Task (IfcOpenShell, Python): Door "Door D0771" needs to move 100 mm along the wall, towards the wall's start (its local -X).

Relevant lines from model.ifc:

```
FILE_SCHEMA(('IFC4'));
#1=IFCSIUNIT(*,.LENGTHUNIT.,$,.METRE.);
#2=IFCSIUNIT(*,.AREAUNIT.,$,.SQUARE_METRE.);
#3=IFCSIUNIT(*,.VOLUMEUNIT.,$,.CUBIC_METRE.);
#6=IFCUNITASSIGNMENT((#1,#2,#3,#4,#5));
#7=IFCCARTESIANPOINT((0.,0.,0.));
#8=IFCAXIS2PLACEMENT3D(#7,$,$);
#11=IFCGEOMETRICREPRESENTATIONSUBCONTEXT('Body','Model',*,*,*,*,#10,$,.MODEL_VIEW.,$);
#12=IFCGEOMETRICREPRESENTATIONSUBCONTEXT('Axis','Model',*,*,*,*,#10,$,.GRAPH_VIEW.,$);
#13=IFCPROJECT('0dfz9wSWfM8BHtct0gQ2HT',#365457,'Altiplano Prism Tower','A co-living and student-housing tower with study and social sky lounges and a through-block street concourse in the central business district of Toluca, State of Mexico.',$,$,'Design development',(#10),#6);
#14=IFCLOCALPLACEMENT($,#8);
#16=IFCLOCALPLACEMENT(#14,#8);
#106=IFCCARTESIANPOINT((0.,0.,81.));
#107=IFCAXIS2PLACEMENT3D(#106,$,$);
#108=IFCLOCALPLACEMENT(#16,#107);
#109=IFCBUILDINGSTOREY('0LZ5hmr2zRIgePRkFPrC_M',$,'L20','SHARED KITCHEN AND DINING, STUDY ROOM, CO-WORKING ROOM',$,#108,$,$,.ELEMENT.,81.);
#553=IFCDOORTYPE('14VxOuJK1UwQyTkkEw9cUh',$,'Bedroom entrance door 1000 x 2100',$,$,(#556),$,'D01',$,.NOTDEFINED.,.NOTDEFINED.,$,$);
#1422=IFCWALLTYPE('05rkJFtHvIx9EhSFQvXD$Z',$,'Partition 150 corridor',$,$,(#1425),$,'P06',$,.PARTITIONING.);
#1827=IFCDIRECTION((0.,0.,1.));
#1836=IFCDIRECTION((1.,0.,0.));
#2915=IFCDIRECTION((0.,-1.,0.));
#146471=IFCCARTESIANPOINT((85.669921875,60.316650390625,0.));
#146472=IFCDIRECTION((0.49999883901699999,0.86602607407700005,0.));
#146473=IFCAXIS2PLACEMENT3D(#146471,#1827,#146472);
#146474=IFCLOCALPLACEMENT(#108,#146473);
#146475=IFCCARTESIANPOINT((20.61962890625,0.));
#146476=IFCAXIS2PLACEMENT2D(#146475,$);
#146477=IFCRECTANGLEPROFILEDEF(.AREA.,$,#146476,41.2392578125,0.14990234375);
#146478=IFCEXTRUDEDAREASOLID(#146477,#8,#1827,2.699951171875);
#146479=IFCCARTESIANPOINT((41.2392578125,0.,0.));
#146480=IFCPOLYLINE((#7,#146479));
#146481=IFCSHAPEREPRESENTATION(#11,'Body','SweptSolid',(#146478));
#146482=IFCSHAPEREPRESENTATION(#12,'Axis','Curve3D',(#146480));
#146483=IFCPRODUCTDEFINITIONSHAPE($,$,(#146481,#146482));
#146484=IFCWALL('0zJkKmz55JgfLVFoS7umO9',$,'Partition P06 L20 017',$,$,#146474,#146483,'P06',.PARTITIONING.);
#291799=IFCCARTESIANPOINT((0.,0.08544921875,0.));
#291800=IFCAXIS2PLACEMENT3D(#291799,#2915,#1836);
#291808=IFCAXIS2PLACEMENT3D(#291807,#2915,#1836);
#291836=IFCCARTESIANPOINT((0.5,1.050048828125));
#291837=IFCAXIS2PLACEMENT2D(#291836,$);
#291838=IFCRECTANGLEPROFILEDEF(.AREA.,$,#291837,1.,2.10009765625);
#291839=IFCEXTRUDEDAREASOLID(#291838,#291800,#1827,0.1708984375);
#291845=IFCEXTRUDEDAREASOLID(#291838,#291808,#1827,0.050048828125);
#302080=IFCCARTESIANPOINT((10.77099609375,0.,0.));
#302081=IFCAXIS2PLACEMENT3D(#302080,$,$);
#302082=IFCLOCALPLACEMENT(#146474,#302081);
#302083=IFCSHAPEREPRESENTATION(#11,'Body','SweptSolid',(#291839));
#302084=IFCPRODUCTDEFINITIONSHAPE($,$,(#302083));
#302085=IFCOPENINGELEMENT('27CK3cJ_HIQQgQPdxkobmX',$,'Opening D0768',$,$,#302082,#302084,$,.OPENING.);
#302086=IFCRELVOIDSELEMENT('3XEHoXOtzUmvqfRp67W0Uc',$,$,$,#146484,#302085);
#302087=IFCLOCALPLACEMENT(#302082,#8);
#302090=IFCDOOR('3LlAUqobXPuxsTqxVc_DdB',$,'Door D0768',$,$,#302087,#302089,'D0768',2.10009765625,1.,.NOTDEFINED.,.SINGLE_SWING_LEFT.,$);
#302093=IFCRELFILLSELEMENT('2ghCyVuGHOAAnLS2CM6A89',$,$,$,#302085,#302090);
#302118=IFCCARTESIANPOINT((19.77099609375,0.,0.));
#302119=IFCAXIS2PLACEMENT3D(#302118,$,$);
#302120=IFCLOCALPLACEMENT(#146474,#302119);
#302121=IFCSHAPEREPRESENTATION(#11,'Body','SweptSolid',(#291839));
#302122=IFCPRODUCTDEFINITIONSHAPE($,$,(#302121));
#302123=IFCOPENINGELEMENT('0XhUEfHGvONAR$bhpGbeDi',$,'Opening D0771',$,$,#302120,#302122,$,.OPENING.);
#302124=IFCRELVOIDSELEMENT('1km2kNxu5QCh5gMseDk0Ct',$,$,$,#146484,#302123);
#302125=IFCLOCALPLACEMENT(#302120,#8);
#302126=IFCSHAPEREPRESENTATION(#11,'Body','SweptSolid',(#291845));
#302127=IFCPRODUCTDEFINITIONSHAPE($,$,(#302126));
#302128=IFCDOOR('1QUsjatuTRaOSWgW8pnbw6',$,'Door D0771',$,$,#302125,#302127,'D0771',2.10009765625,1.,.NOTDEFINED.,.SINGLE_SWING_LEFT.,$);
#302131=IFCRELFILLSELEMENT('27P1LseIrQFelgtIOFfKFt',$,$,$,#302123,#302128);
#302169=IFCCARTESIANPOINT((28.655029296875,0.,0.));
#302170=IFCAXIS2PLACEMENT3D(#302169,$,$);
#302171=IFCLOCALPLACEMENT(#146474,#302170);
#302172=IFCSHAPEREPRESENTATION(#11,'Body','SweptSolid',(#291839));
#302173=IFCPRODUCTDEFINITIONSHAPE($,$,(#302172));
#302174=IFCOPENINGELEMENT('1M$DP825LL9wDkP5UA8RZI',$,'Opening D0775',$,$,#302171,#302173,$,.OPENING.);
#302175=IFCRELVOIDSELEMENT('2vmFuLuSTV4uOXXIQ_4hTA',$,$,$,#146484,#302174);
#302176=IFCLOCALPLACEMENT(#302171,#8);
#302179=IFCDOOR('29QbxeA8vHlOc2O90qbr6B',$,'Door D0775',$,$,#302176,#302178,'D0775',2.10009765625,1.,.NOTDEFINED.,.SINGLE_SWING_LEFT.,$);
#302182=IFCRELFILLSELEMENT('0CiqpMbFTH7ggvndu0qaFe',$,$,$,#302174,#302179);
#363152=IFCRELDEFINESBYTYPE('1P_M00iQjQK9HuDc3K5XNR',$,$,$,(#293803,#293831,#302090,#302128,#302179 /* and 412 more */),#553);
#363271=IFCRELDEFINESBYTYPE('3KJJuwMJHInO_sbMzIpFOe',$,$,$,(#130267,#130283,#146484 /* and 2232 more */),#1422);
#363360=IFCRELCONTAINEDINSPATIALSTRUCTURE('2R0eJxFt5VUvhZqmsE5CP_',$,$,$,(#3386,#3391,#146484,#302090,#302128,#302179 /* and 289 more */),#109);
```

```python
import ifcopenshell
import ifcopenshell.api.geometry
import ifcopenshell.util.placement
import ifcopenshell.util.unit

model = ifcopenshell.open("model.ifc")
unit_scale = ifcopenshell.util.unit.calculate_unit_scale(model)

door = model.by_guid("1QUsjatuTRaOSWgW8pnbw6")
opening = door.FillsVoids[0].RelatingOpeningElement
wall = opening.VoidsElements[0].RelatingBuildingElement

wall_matrix = ifcopenshell.util.placement.get_local_placement(wall.ObjectPlacement)
shift = wall_matrix[:3, 0] * -0.1 / unit_scale
before = ifcopenshell.util.placement.get_local_placement(door.ObjectPlacement)[:3, 3].copy()

# The door is placed relative to its opening, so it follows when the opening moves.
matrix = ifcopenshell.util.placement.get_local_placement(opening.ObjectPlacement)
matrix[:3, 3] += shift
ifcopenshell.api.geometry.edit_object_placement(
    model, product=opening, matrix=matrix, is_si=False, should_transform_children=True
)

after = ifcopenshell.util.placement.get_local_placement(door.ObjectPlacement)[:3, 3]
print("door moved by", (after - before).round(3) + 0.0)

model.write("model_v2.ifc")
```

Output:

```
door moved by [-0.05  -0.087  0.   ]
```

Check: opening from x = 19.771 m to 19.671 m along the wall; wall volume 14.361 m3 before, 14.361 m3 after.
